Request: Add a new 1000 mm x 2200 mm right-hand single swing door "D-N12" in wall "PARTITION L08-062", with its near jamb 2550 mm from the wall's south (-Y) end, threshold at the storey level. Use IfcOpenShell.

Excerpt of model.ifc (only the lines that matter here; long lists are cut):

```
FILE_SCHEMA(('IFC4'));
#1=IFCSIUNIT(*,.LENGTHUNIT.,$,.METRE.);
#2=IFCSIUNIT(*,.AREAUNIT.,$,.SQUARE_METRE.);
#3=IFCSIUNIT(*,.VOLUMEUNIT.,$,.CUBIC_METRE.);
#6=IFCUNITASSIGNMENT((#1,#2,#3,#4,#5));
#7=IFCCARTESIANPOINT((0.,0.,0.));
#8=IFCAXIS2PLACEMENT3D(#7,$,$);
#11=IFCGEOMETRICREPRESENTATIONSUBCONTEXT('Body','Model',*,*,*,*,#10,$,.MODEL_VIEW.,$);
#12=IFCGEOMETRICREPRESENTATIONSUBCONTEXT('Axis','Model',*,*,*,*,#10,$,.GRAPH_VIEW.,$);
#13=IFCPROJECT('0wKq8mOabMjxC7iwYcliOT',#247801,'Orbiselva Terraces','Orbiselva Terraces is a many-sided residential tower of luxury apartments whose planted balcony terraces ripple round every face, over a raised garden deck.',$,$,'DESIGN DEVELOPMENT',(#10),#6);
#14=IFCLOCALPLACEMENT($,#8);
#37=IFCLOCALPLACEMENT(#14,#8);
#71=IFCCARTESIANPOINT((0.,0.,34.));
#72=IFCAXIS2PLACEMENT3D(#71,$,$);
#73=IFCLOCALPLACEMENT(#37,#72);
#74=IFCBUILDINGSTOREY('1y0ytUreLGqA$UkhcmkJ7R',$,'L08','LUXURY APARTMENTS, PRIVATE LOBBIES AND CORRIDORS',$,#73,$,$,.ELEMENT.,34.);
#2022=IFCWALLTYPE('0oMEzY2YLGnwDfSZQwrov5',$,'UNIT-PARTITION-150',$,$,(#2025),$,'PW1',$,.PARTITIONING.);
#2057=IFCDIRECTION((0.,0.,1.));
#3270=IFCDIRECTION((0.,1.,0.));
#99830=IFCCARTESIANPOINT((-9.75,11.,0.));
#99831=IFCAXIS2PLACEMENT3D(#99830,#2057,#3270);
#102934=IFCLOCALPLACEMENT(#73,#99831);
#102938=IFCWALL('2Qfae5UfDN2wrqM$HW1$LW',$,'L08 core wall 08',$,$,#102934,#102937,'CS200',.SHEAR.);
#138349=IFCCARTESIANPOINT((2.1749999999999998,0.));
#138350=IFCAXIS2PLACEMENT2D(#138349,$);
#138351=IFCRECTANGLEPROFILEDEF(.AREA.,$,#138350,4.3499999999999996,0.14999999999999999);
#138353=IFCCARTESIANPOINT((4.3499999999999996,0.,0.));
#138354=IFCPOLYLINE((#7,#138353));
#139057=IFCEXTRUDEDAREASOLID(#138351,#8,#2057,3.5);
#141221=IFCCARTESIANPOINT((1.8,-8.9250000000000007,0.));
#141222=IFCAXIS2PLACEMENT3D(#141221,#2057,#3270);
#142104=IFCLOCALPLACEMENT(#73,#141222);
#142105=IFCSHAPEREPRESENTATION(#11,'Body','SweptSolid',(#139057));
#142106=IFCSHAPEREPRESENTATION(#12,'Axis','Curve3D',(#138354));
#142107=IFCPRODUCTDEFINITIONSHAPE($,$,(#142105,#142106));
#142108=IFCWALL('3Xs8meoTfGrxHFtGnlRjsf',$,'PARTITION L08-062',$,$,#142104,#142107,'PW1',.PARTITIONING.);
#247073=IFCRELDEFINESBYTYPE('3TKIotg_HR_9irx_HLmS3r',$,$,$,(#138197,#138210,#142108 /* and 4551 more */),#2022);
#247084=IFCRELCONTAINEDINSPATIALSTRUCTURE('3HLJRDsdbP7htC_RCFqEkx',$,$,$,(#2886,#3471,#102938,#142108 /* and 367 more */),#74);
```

```python
import numpy as np
import ifcopenshell
import ifcopenshell.api.feature
import ifcopenshell.api.geometry
import ifcopenshell.api.root
import ifcopenshell.api.spatial
import ifcopenshell.geom
import ifcopenshell.util.element
import ifcopenshell.util.placement
import ifcopenshell.util.representation
import ifcopenshell.util.shape
import ifcopenshell.util.unit

model = ifcopenshell.open("model.ifc")
unit_scale = ifcopenshell.util.unit.calculate_unit_scale(model)
settings = ifcopenshell.geom.settings()


def volume(element):
    """Net volume in cubic metres, openings subtracted."""
    shape = ifcopenshell.geom.create_shape(settings, element)
    return ifcopenshell.util.shape.get_volume(shape.geometry)


wall = model.by_guid("3Xs8meoTfGrxHFtGnlRjsf")
storey = ifcopenshell.util.element.get_container(wall, ifc_class="IfcBuildingStorey")
context = ifcopenshell.util.representation.get_context(model, "Model", "Body", "MODEL_VIEW")
before = volume(wall)

width, height, from_end, sill = 1, 2.2, 2.55, 0.0  # metres

# The wall runs along its own X axis, and the end named is its -X end.
wall_shape = ifcopenshell.geom.create_shape(settings, wall)
x, y, z = ifcopenshell.util.shape.get_vertices(wall_shape.geometry).T
start = x.min() + from_end
face, thickness = float(y.min()), float(y.max() - y.min())
wall_matrix = ifcopenshell.util.placement.get_local_placement(wall.ObjectPlacement)
level = ifcopenshell.util.placement.get_local_placement(storey.ObjectPlacement)[2, 3]


def in_wall(x, y):
    """Placement at x, y metres in the wall's axes, at sill height."""
    matrix = wall_matrix.copy()
    matrix[:, 3] = wall_matrix @ np.array([x / unit_scale, y / unit_scale, 0.0, 1.0])
    matrix[2, 3] = level + sill / unit_scale
    return matrix


# Opening: a box that overshoots both wall faces by 50 mm.
opening = ifcopenshell.api.root.create_entity(model, ifc_class="IfcOpeningElement", predefined_type="OPENING")
box = ifcopenshell.api.geometry.add_wall_representation(
    model, context=context, length=width, height=height, thickness=thickness + 0.1
)
ifcopenshell.api.geometry.assign_representation(model, product=opening, representation=box)
ifcopenshell.api.geometry.edit_object_placement(model, product=opening, matrix=in_wall(start, face - 0.05), is_si=False)
ifcopenshell.api.feature.add_feature(model, feature=opening, element=wall)

door = ifcopenshell.api.root.create_entity(model, ifc_class="IfcDoor", name="D-N12", predefined_type="DOOR")
door.OverallWidth, door.OverallHeight = width / unit_scale, height / unit_scale
door.OperationType = "SINGLE_SWING_RIGHT"
body = ifcopenshell.api.geometry.add_door_representation(
    model,
    context=context,
    overall_width=door.OverallWidth,
    overall_height=door.OverallHeight,
    operation_type="SINGLE_SWING_RIGHT",
    lining_properties={"LiningDepth": thickness / unit_scale, "ThresholdDepth": thickness / unit_scale},
)
ifcopenshell.api.geometry.assign_representation(model, product=door, representation=body)
ifcopenshell.api.spatial.assign_container(model, products=[door], relating_structure=storey)
ifcopenshell.api.feature.add_filling(model, opening=opening, element=door)

# The lining spans the wall, so the door starts at the wall face.
ifcopenshell.api.geometry.edit_object_placement(model, product=door, matrix=in_wall(start, face), is_si=False)

after = volume(wall)

print(f"wall volume {before:.3f} -> {after:.3f} m3")

model.write("model_v2.ifc")
```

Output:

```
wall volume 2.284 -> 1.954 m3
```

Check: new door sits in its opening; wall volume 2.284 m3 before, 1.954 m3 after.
